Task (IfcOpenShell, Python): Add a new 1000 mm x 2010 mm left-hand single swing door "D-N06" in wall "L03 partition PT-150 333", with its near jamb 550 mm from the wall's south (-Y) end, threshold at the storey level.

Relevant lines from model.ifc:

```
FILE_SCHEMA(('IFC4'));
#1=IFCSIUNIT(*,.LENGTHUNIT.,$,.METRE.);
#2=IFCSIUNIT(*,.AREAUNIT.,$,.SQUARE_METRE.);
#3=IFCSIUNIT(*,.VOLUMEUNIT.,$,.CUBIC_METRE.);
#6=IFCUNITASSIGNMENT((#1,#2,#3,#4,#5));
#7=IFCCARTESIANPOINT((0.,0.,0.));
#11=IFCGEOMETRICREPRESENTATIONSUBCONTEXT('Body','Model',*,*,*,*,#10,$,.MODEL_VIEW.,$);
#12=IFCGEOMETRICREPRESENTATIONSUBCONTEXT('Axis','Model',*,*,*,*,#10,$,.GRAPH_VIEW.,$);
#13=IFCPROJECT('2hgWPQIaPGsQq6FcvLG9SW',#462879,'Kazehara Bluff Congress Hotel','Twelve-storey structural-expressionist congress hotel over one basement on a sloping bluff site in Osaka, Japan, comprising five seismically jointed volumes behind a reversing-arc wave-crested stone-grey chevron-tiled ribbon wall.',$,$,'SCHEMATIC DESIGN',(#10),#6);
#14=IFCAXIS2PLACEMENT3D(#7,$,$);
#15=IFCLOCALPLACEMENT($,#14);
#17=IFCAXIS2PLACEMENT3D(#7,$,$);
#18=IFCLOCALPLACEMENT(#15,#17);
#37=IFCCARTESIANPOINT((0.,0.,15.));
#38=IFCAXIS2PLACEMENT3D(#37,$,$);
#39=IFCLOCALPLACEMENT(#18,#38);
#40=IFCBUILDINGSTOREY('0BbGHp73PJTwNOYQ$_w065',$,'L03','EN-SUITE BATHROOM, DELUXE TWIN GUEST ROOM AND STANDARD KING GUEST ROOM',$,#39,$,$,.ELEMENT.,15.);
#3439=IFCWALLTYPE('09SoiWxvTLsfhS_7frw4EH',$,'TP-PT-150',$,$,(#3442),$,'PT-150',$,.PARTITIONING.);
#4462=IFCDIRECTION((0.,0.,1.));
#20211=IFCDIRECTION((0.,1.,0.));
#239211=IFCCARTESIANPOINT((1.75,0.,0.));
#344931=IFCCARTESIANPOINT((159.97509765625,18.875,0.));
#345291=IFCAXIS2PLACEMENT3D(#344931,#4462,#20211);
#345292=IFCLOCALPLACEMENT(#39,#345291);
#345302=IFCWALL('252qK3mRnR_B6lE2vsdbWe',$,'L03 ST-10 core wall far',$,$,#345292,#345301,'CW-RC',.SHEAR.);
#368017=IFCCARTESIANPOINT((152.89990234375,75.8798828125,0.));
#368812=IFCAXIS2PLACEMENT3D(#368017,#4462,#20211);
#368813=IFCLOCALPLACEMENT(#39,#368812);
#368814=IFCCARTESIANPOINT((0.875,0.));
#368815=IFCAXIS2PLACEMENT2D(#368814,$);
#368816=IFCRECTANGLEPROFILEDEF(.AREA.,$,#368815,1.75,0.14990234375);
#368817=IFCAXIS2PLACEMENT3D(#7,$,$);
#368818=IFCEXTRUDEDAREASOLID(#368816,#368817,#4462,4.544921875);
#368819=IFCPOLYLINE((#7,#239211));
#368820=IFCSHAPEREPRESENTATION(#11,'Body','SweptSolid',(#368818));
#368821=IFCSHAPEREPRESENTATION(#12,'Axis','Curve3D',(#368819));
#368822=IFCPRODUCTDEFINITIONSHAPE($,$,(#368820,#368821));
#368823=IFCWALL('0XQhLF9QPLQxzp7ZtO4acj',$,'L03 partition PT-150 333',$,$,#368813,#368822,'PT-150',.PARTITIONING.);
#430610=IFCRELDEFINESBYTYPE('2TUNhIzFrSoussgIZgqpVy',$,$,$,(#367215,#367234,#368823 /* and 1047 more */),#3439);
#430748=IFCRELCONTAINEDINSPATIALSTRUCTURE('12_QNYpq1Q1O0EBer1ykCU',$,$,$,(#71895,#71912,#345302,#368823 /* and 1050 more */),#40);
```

```python
import numpy as np
import ifcopenshell
import ifcopenshell.api.feature
import ifcopenshell.api.geometry
import ifcopenshell.api.root
import ifcopenshell.api.spatial
import ifcopenshell.geom
import ifcopenshell.util.element
import ifcopenshell.util.placement
import ifcopenshell.util.representation
import ifcopenshell.util.shape
import ifcopenshell.util.unit

model = ifcopenshell.open("model.ifc")
unit_scale = ifcopenshell.util.unit.calculate_unit_scale(model)
settings = ifcopenshell.geom.settings()


def volume(element):
    """Net volume in cubic metres, openings subtracted."""
    shape = ifcopenshell.geom.create_shape(settings, element)
    return ifcopenshell.util.shape.get_volume(shape.geometry)


wall = model.by_guid("0XQhLF9QPLQxzp7ZtO4acj")
storey = ifcopenshell.util.element.get_container(wall, ifc_class="IfcBuildingStorey")
context = ifcopenshell.util.representation.get_context(model, "Model", "Body", "MODEL_VIEW")
before = volume(wall)

width, height, from_end, sill = 1, 2.01, 0.55, 0.0  # metres

# The wall runs along its own X axis, and the end named is its -X end.
wall_shape = ifcopenshell.geom.create_shape(settings, wall)
x, y, z = ifcopenshell.util.shape.get_vertices(wall_shape.geometry).T
start = x.min() + from_end
face, thickness = float(y.min()), float(y.max() - y.min())
wall_matrix = ifcopenshell.util.placement.get_local_placement(wall.ObjectPlacement)
level = ifcopenshell.util.placement.get_local_placement(storey.ObjectPlacement)[2, 3]


def in_wall(x, y):
    """Placement at x, y metres in the wall's axes, at sill height."""
    matrix = wall_matrix.copy()
    matrix[:, 3] = wall_matrix @ np.array([x / unit_scale, y / unit_scale, 0.0, 1.0])
    matrix[2, 3] = level + sill / unit_scale
    return matrix


# Opening: a box that overshoots both wall faces by 50 mm.
opening = ifcopenshell.api.root.create_entity(model, ifc_class="IfcOpeningElement", predefined_type="OPENING")
box = ifcopenshell.api.geometry.add_wall_representation(
    model, context=context, length=width, height=height, thickness=thickness + 0.1
)
ifcopenshell.api.geometry.assign_representation(model, product=opening, representation=box)
ifcopenshell.api.geometry.edit_object_placement(model, product=opening, matrix=in_wall(start, face - 0.05), is_si=False)
ifcopenshell.api.feature.add_feature(model, feature=opening, element=wall)

door = ifcopenshell.api.root.create_entity(model, ifc_class="IfcDoor", name="D-N06", predefined_type="DOOR")
door.OverallWidth, door.OverallHeight = width / unit_scale, height / unit_scale
door.OperationType = "SINGLE_SWING_LEFT"
body = ifcopenshell.api.geometry.add_door_representation(
    model,
    context=context,
    overall_width=door.OverallWidth,
    overall_height=door.OverallHeight,
    operation_type="SINGLE_SWING_LEFT",
    lining_properties={"LiningDepth": thickness / unit_scale, "ThresholdDepth": thickness / unit_scale},
)
ifcopenshell.api.geometry.assign_representation(model, product=door, representation=body)
ifcopenshell.api.spatial.assign_container(model, products=[door], relating_structure=storey)
ifcopenshell.api.feature.add_filling(model, opening=opening, element=door)

# The lining spans the wall, so the door starts at the wall face.
ifcopenshell.api.geometry.edit_object_placement(model, product=door, matrix=in_wall(start, face), is_si=False)

after = volume(wall)

print(f"wall volume {before:.3f} -> {after:.3f} m3")

model.write("model_v2.ifc")
```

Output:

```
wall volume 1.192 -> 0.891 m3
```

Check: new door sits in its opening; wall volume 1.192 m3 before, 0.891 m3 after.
